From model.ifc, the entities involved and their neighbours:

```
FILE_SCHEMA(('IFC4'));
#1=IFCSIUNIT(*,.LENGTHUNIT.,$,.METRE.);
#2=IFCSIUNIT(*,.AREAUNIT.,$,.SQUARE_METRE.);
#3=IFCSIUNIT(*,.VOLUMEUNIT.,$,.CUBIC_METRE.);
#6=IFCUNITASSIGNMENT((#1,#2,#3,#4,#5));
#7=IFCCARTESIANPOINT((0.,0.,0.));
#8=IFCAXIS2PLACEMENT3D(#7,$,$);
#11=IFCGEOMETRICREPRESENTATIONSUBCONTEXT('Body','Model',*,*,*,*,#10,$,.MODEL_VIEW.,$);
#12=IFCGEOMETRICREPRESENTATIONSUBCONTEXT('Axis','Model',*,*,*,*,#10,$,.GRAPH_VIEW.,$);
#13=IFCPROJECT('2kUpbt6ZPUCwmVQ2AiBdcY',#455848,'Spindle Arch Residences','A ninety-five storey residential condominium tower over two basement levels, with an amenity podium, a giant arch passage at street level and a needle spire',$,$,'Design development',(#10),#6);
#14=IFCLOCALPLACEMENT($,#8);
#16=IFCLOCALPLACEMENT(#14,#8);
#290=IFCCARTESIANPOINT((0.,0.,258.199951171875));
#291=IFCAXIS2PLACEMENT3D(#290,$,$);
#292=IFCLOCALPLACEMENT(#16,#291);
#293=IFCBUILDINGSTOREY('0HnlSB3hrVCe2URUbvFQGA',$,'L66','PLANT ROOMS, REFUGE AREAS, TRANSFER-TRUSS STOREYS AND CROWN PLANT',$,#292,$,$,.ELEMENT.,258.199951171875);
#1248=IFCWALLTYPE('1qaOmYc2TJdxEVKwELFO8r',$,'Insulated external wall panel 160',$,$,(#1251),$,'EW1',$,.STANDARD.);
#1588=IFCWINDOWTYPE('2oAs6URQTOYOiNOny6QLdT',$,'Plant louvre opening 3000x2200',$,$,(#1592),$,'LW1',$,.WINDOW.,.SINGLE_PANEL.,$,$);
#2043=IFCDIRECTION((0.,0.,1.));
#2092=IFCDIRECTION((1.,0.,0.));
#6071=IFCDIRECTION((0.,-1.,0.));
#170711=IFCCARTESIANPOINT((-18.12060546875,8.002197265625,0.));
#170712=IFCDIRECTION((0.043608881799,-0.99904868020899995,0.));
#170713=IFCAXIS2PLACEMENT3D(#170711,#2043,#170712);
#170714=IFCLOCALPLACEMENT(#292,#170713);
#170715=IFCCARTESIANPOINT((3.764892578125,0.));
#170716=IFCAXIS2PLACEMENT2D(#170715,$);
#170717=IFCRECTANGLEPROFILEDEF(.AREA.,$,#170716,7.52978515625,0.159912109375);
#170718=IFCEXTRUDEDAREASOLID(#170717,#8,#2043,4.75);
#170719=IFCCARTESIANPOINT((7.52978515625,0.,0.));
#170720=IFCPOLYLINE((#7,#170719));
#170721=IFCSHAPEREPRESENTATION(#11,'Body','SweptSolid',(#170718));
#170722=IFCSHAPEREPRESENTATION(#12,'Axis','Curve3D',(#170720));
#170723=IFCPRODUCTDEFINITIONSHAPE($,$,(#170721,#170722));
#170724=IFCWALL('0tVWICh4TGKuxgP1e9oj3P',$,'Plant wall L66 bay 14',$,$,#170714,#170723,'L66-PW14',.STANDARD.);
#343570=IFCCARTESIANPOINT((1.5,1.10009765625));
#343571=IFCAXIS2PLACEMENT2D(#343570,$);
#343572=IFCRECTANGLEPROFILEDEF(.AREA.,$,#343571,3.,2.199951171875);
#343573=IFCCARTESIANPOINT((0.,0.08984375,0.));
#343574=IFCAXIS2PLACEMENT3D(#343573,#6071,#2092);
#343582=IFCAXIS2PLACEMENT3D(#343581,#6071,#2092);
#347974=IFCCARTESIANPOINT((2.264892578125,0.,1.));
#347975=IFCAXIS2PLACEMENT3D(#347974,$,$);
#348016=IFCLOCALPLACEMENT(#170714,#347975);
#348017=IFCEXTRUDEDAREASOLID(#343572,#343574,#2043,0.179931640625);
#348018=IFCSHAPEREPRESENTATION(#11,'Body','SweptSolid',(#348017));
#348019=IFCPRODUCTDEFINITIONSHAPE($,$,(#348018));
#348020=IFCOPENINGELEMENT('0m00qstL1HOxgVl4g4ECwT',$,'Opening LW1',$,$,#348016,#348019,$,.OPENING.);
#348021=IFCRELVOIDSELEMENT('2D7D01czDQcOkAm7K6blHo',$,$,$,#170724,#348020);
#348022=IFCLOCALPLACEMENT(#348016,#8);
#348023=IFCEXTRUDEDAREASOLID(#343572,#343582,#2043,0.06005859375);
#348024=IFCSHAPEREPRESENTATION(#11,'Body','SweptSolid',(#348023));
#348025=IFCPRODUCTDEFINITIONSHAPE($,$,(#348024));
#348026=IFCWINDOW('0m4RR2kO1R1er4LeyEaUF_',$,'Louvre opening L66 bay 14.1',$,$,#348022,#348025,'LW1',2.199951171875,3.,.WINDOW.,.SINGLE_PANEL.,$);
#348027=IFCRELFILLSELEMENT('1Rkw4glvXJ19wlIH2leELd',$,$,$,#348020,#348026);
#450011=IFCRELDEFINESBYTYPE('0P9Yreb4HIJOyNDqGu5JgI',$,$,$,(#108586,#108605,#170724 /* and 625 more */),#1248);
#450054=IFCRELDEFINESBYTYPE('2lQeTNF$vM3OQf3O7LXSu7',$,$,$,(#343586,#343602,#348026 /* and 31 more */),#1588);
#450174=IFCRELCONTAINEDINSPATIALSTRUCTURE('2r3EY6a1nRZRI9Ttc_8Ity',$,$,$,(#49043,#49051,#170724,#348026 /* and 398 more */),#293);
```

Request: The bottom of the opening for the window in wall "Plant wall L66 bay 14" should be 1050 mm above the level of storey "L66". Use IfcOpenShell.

```python
import numpy as np
import ifcopenshell
import ifcopenshell.api.geometry
import ifcopenshell.geom
import ifcopenshell.util.element
import ifcopenshell.util.placement
import ifcopenshell.util.shape
import ifcopenshell.util.unit

model = ifcopenshell.open("model.ifc")
unit_scale = ifcopenshell.util.unit.calculate_unit_scale(model)

window = model.by_guid("0m4RR2kO1R1er4LeyEaUF_")
opening = window.FillsVoids[0].RelatingOpeningElement
storey = ifcopenshell.util.element.get_container(window, ifc_class="IfcBuildingStorey")
level = ifcopenshell.util.placement.get_local_placement(storey.ObjectPlacement)[2, 3]

# The opening's origin need not be at the sill, so measure its lowest point.
shape = ifcopenshell.geom.create_shape(ifcopenshell.geom.settings(), opening)
bottom = ifcopenshell.util.shape.get_shape_bottom_elevation(shape, shape.geometry) / unit_scale
dz = level + 1.05 - bottom

shift = np.array([0.0, 0.0, dz])
# The window is placed relative to its opening, so it follows when the opening moves.
matrix = ifcopenshell.util.placement.get_local_placement(opening.ObjectPlacement)
matrix[:3, 3] += shift
ifcopenshell.api.geometry.edit_object_placement(
    model, product=opening, matrix=matrix, is_si=False, should_transform_children=True
)

print(f"moved by {dz * unit_scale:+.3f} m")

model.write("model_v2.ifc")
```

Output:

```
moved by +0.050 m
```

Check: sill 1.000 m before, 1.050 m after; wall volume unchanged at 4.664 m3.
